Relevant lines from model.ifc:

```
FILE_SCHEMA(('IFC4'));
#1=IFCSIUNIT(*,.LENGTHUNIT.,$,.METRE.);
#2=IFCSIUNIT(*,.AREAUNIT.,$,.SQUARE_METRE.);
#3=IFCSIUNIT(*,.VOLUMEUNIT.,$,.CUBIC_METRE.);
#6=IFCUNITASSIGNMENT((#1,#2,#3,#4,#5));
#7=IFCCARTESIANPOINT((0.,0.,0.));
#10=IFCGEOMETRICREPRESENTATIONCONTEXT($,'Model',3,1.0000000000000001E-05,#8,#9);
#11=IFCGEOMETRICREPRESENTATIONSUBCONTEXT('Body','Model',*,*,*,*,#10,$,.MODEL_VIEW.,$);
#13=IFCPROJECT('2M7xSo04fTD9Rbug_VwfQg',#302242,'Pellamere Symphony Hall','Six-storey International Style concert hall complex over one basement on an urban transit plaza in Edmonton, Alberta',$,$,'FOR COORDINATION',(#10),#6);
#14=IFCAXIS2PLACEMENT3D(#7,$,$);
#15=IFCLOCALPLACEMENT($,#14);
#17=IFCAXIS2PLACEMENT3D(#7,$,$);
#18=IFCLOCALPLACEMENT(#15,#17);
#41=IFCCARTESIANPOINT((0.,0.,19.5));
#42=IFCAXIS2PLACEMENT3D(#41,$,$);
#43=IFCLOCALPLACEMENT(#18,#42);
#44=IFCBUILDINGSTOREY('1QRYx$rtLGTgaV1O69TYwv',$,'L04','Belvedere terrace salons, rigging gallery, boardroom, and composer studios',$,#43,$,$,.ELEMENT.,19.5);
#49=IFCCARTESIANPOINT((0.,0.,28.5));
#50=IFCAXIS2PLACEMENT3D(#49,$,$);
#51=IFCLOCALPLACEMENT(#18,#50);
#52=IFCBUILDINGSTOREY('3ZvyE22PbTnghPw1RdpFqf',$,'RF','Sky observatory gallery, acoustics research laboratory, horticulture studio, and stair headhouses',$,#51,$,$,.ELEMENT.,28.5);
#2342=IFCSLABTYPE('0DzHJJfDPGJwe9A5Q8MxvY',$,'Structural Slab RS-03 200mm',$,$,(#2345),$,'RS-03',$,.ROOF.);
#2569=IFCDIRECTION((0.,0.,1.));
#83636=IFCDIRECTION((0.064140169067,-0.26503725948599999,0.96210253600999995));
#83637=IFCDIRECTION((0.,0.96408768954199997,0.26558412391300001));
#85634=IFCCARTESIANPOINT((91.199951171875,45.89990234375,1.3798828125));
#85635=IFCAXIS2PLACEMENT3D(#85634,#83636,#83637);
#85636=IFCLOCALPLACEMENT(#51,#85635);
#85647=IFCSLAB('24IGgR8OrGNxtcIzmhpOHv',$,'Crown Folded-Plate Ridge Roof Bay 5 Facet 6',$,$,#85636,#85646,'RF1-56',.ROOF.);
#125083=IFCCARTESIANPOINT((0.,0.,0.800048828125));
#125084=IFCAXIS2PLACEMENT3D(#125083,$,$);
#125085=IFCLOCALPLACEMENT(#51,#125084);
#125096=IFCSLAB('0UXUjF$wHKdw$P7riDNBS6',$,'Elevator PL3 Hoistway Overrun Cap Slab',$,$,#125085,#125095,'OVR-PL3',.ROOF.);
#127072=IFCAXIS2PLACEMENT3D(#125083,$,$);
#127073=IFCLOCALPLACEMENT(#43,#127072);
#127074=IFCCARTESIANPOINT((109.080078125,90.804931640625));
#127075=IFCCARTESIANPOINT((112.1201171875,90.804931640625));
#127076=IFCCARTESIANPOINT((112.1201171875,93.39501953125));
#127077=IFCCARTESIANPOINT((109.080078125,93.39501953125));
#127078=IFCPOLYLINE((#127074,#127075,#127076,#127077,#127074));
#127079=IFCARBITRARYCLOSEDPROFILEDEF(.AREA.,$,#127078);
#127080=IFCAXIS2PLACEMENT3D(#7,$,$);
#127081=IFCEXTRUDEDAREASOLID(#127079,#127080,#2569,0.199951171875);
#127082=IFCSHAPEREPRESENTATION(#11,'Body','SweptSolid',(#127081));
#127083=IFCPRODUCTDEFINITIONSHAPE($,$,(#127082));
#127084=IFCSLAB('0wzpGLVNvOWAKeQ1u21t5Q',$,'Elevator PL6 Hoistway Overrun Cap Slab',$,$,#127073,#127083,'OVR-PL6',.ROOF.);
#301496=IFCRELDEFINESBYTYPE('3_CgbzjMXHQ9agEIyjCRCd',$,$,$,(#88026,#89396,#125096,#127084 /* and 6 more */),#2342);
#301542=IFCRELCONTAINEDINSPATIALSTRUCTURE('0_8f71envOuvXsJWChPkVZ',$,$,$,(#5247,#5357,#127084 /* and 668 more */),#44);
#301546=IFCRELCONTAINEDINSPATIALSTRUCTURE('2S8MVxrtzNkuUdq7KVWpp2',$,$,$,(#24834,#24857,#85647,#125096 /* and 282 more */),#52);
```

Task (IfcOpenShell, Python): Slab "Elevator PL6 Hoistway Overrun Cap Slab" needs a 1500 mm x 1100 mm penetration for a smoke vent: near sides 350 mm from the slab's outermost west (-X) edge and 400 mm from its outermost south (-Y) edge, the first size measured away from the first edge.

```python
import numpy as np
import ifcopenshell
import ifcopenshell.api.feature
import ifcopenshell.api.geometry
import ifcopenshell.api.root
import ifcopenshell.geom
import ifcopenshell.util.placement
import ifcopenshell.util.representation
import ifcopenshell.util.shape
import ifcopenshell.util.unit

model = ifcopenshell.open("model.ifc")
unit_scale = ifcopenshell.util.unit.calculate_unit_scale(model)
settings = ifcopenshell.geom.settings()


def volume(element):
    """Net volume in cubic metres, openings subtracted."""
    shape = ifcopenshell.geom.create_shape(settings, element)
    return ifcopenshell.util.shape.get_volume(shape.geometry)


slab = model.by_id(127084)
before = volume(slab)

# Extent in the slab's own axes, in metres. The edges named are its -X and -Y sides.
slab_shape = ifcopenshell.geom.create_shape(settings, slab)
vertices = ifcopenshell.util.shape.get_vertices(slab_shape.geometry)
x_min, y_min, bottom = vertices.min(axis=0)
top = vertices[:, 2].max()

opening = ifcopenshell.api.root.create_entity(model, ifc_class="IfcOpeningElement", name="Smoke vent opening", predefined_type="OPENING")
context = ifcopenshell.util.representation.get_context(model, "Model", "Body", "MODEL_VIEW")
width, depth = 1.5, 1.1
outline = [(0.0, 0.0), (width, 0.0), (width, depth), (0.0, depth), (0.0, 0.0)]
# Overshoot both faces by 50 mm so the cut is clean.
shape = ifcopenshell.api.geometry.add_slab_representation(
    model, context=context, depth=top - bottom + 0.1, polyline=outline
)
ifcopenshell.api.geometry.assign_representation(model, product=opening, representation=shape)

matrix = ifcopenshell.util.placement.get_local_placement(slab.ObjectPlacement)
matrix[:, 3] = matrix @ np.append(np.array([x_min + 0.35, y_min + 0.4, bottom - 0.05]) / unit_scale, 1.0)
ifcopenshell.api.geometry.edit_object_placement(model, product=opening, matrix=matrix, is_si=False)
ifcopenshell.api.feature.add_feature(model, feature=opening, element=slab)

after = volume(slab)

print(f"slab volume {before:.3f} -> {after:.3f} m3")

model.write("model_edited.ifc")
```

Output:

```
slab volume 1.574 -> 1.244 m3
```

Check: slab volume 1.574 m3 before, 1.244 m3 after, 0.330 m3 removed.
